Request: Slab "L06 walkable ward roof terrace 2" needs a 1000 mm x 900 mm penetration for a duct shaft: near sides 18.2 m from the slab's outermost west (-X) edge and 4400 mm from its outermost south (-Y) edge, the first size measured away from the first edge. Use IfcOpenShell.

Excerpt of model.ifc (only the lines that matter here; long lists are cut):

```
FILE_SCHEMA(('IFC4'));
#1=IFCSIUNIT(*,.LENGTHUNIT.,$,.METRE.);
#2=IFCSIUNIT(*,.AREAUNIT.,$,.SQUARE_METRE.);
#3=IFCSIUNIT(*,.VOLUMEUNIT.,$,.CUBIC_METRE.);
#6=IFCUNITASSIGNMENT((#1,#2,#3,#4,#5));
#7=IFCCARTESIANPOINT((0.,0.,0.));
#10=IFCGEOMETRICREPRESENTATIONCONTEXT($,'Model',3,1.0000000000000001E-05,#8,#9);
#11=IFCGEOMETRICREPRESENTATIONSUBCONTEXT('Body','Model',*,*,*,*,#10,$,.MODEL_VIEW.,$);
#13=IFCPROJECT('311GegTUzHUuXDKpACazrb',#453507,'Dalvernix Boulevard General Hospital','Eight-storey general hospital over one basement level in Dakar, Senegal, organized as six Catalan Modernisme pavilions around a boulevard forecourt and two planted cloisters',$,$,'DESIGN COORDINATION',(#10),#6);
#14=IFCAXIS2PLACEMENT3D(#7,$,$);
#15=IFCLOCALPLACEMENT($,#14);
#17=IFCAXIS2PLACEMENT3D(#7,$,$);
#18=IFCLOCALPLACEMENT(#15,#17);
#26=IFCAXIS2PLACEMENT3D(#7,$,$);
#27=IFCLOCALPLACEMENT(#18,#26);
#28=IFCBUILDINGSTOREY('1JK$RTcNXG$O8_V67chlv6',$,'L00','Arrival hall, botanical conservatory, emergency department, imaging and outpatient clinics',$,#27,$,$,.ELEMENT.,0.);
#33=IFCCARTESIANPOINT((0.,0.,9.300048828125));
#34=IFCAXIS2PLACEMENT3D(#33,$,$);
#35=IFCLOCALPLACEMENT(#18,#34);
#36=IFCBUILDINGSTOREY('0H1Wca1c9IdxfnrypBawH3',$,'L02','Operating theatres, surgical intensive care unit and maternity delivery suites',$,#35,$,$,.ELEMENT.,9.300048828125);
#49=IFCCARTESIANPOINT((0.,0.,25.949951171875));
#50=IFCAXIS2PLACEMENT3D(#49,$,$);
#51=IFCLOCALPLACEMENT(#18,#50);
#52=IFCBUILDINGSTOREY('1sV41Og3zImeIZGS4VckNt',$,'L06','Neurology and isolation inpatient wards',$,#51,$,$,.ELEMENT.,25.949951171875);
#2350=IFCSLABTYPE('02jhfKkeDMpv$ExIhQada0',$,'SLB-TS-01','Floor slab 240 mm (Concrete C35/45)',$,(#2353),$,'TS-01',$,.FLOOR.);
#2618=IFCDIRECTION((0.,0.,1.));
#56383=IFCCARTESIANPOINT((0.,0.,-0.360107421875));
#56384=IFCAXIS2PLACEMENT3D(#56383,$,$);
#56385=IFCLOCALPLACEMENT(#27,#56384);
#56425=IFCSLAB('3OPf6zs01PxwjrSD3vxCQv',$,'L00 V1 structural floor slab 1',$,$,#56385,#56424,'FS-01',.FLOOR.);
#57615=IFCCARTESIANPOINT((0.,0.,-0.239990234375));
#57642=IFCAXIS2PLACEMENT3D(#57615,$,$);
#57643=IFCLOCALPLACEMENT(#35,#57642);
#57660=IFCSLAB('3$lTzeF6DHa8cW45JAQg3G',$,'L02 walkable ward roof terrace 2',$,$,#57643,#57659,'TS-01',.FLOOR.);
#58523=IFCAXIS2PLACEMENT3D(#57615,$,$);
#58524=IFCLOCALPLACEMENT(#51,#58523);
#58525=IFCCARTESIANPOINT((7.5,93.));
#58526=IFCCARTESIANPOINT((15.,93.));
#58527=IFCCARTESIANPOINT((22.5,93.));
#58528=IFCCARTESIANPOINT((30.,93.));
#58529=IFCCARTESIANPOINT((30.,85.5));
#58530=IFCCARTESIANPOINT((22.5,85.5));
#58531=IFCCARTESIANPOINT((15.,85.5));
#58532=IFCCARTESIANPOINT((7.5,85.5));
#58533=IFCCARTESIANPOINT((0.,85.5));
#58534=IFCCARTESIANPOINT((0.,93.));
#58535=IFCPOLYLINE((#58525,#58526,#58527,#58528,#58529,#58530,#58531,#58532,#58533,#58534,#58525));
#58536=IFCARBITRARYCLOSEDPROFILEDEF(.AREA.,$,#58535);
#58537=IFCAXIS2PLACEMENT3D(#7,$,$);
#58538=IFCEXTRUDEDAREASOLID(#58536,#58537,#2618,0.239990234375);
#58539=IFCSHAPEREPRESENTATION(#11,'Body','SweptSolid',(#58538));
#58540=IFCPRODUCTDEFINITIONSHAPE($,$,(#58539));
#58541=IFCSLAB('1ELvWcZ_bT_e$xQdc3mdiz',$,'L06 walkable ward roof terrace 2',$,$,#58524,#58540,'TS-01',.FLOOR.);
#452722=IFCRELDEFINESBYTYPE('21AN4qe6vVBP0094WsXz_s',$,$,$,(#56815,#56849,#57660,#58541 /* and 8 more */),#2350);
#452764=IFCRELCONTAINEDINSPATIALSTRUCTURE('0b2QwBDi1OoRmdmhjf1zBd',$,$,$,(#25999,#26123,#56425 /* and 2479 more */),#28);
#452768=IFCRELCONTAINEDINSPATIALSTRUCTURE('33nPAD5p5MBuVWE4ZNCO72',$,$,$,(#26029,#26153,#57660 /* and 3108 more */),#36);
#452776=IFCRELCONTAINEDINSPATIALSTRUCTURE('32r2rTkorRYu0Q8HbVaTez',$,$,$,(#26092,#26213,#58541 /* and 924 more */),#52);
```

```python
import numpy as np
import ifcopenshell
import ifcopenshell.api.feature
import ifcopenshell.api.geometry
import ifcopenshell.api.root
import ifcopenshell.geom
import ifcopenshell.util.placement
import ifcopenshell.util.representation
import ifcopenshell.util.shape
import ifcopenshell.util.unit

model = ifcopenshell.open("model.ifc")
unit_scale = ifcopenshell.util.unit.calculate_unit_scale(model)
settings = ifcopenshell.geom.settings()


def volume(element):
    """Net volume in cubic metres, openings subtracted."""
    shape = ifcopenshell.geom.create_shape(settings, element)
    return ifcopenshell.util.shape.get_volume(shape.geometry)


slab = model.by_guid("1ELvWcZ_bT_e$xQdc3mdiz")
before = volume(slab)

# Extent in the slab's own axes, in metres. The edges named are its -X and -Y sides.
slab_shape = ifcopenshell.geom.create_shape(settings, slab)
vertices = ifcopenshell.util.shape.get_vertices(slab_shape.geometry)
x_min, y_min, bottom = vertices.min(axis=0)
top = vertices[:, 2].max()

opening = ifcopenshell.api.root.create_entity(model, ifc_class="IfcOpeningElement", name="Duct shaft opening", predefined_type="OPENING")
context = ifcopenshell.util.representation.get_context(model, "Model", "Body", "MODEL_VIEW")
width, depth = 1, 0.9
outline = [(0.0, 0.0), (width, 0.0), (width, depth), (0.0, depth), (0.0, 0.0)]
# Overshoot both faces by 50 mm so the cut is clean.
shape = ifcopenshell.api.geometry.add_slab_representation(
    model, context=context, depth=top - bottom + 0.1, polyline=outline
)
ifcopenshell.api.geometry.assign_representation(model, product=opening, representation=shape)

matrix = ifcopenshell.util.placement.get_local_placement(slab.ObjectPlacement)
matrix[:, 3] = matrix @ np.append(np.array([x_min + 18.2, y_min + 4.4, bottom - 0.05]) / unit_scale, 1.0)
ifcopenshell.api.geometry.edit_object_placement(model, product=opening, matrix=matrix, is_si=False)
ifcopenshell.api.feature.add_feature(model, feature=opening, element=slab)

after = volume(slab)

print(f"slab volume {before:.3f} -> {after:.3f} m3")

model.write("model_updated.ifc")
```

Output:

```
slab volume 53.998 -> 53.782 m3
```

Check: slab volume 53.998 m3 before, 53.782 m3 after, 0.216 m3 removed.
